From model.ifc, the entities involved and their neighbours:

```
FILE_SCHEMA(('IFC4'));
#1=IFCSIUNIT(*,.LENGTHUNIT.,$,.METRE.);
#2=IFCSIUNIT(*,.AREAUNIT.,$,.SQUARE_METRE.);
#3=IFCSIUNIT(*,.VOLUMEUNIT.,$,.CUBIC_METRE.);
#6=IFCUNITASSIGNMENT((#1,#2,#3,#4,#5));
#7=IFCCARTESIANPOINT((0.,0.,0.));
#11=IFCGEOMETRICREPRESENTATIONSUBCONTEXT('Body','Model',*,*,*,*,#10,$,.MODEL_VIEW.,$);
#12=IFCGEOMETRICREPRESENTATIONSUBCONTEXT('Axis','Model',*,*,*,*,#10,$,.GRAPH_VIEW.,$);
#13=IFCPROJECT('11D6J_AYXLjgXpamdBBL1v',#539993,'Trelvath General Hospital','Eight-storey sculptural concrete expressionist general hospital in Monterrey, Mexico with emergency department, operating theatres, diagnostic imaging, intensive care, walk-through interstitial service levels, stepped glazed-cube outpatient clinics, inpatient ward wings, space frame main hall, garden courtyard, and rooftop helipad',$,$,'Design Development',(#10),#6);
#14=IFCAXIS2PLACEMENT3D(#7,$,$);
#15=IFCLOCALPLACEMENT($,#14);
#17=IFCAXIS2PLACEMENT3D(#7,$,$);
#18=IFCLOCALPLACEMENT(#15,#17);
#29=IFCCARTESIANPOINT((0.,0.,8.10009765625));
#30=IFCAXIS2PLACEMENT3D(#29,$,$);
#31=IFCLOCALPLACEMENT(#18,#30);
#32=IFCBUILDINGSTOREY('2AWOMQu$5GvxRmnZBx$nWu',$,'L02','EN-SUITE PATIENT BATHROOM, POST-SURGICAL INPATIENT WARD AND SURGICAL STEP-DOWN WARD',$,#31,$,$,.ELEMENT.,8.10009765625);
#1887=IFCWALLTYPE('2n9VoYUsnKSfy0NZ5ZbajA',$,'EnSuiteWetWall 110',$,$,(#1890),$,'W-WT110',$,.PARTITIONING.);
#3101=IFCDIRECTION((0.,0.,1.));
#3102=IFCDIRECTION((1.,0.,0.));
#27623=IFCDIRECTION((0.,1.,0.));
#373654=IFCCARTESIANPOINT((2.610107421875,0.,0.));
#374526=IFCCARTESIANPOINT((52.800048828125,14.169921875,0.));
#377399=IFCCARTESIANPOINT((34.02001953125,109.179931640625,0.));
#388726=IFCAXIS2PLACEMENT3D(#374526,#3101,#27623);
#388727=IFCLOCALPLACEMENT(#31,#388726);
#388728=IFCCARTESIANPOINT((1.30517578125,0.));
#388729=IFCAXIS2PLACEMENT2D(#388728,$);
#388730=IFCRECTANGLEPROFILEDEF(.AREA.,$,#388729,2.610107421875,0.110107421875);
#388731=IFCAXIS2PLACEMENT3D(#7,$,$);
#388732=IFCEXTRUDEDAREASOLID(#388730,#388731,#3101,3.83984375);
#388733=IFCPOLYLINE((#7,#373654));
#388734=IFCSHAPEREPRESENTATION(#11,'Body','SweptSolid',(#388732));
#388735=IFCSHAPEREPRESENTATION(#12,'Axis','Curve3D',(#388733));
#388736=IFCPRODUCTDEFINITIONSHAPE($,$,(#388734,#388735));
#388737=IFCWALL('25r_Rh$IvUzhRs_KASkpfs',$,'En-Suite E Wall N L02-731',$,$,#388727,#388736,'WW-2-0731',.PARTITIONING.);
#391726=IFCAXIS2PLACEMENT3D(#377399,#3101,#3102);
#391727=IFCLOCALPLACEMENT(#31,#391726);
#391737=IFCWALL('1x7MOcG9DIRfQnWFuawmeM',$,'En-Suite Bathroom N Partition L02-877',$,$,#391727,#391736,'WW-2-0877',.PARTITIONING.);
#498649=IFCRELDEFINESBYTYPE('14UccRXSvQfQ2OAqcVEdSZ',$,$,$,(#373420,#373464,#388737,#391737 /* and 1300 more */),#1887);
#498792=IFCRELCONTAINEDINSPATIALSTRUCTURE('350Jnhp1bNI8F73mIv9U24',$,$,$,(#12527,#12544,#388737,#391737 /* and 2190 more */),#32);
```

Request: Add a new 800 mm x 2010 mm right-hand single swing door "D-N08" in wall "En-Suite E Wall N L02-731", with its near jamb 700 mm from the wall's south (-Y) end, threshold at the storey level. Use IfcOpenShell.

```python
import numpy as np
import ifcopenshell
import ifcopenshell.api.feature
import ifcopenshell.api.geometry
import ifcopenshell.api.root
import ifcopenshell.api.spatial
import ifcopenshell.geom
import ifcopenshell.util.element
import ifcopenshell.util.placement
import ifcopenshell.util.representation
import ifcopenshell.util.shape
import ifcopenshell.util.unit

model = ifcopenshell.open("model.ifc")
unit_scale = ifcopenshell.util.unit.calculate_unit_scale(model)
settings = ifcopenshell.geom.settings()


def volume(element):
    """Net volume in cubic metres, openings subtracted."""
    shape = ifcopenshell.geom.create_shape(settings, element)
    return ifcopenshell.util.shape.get_volume(shape.geometry)


wall = model.by_guid("25r_Rh$IvUzhRs_KASkpfs")
storey = ifcopenshell.util.element.get_container(wall, ifc_class="IfcBuildingStorey")
context = ifcopenshell.util.representation.get_context(model, "Model", "Body", "MODEL_VIEW")
before = volume(wall)

width, height, from_end, sill = 0.8, 2.01, 0.7, 0.0  # metres

# The wall runs along its own X axis, and the end named is its -X end.
wall_shape = ifcopenshell.geom.create_shape(settings, wall)
x, y, z = ifcopenshell.util.shape.get_vertices(wall_shape.geometry).T
start = x.min() + from_end
face, thickness = float(y.min()), float(y.max() - y.min())
wall_matrix = ifcopenshell.util.placement.get_local_placement(wall.ObjectPlacement)
level = ifcopenshell.util.placement.get_local_placement(storey.ObjectPlacement)[2, 3]


def in_wall(x, y):
    """Placement at x, y metres in the wall's axes, at sill height."""
    matrix = wall_matrix.copy()
    matrix[:, 3] = wall_matrix @ np.array([x / unit_scale, y / unit_scale, 0.0, 1.0])
    matrix[2, 3] = level + sill / unit_scale
    return matrix


# Opening: a box that overshoots both wall faces by 50 mm.
opening = ifcopenshell.api.root.create_entity(model, ifc_class="IfcOpeningElement", predefined_type="OPENING")
box = ifcopenshell.api.geometry.add_wall_representation(
    model, context=context, length=width, height=height, thickness=thickness + 0.1
)
ifcopenshell.api.geometry.assign_representation(model, product=opening, representation=box)
ifcopenshell.api.geometry.edit_object_placement(model, product=opening, matrix=in_wall(start, face - 0.05), is_si=False)
ifcopenshell.api.feature.add_feature(model, feature=opening, element=wall)

door = ifcopenshell.api.root.create_entity(model, ifc_class="IfcDoor", name="D-N08", predefined_type="DOOR")
door.OverallWidth, door.OverallHeight = width / unit_scale, height / unit_scale
door.OperationType = "SINGLE_SWING_RIGHT"
body = ifcopenshell.api.geometry.add_door_representation(
    model,
    context=context,
    overall_width=door.OverallWidth,
    overall_height=door.OverallHeight,
    operation_type="SINGLE_SWING_RIGHT",
    lining_properties={"LiningDepth": thickness / unit_scale, "ThresholdDepth": thickness / unit_scale},
)
ifcopenshell.api.geometry.assign_representation(model, product=door, representation=body)
ifcopenshell.api.spatial.assign_container(model, products=[door], relating_structure=storey)
ifcopenshell.api.feature.add_filling(model, opening=opening, element=door)

# The lining spans the wall, so the door starts at the wall face.
ifcopenshell.api.geometry.edit_object_placement(model, product=door, matrix=in_wall(start, face), is_si=False)

after = volume(wall)

print(f"wall volume {before:.3f} -> {after:.3f} m3")

model.write("model_updated.ifc")
```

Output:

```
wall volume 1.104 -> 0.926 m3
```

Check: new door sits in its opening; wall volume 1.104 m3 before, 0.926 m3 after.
